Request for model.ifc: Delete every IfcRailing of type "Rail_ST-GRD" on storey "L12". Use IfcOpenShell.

First a look at what the model holds.

```python
import ifcopenshell
import ifcopenshell.util.element

model = ifcopenshell.open("model.ifc")
print(model.schema)
storey = next(s for s in model.by_type("IfcBuildingStorey") if s.Name == "L12")
railings = [e for e in ifcopenshell.util.element.get_decomposition(storey) if e.is_a("IfcRailing")]
seen = {}
for e in railings:
    element_type = ifcopenshell.util.element.get_type(e)
    name = element_type.Name if element_type not in (None, e) else None
    seen[name] = seen.get(name, 0) + 1
for name, count in sorted(seen.items(), key=str):
    print(count, "x", name)
```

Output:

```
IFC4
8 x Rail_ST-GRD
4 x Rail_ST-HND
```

```python
import ifcopenshell
import ifcopenshell.api.root
import ifcopenshell.util.element

model = ifcopenshell.open("model.ifc")

storey = next(s for s in model.by_type("IfcBuildingStorey") if s.Name == "L12")
railings = [e for e in ifcopenshell.util.element.get_decomposition(storey) if e.is_a("IfcRailing")]
targets = [e for e in railings if (t := ifcopenshell.util.element.get_type(e)) not in (None, e) and t.Name == "Rail_ST-GRD"]

for e in targets:
    ifcopenshell.api.root.remove_product(model, product=e)
print(len(targets), "removed")

model.write("model_updated.ifc")
```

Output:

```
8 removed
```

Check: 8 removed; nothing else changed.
